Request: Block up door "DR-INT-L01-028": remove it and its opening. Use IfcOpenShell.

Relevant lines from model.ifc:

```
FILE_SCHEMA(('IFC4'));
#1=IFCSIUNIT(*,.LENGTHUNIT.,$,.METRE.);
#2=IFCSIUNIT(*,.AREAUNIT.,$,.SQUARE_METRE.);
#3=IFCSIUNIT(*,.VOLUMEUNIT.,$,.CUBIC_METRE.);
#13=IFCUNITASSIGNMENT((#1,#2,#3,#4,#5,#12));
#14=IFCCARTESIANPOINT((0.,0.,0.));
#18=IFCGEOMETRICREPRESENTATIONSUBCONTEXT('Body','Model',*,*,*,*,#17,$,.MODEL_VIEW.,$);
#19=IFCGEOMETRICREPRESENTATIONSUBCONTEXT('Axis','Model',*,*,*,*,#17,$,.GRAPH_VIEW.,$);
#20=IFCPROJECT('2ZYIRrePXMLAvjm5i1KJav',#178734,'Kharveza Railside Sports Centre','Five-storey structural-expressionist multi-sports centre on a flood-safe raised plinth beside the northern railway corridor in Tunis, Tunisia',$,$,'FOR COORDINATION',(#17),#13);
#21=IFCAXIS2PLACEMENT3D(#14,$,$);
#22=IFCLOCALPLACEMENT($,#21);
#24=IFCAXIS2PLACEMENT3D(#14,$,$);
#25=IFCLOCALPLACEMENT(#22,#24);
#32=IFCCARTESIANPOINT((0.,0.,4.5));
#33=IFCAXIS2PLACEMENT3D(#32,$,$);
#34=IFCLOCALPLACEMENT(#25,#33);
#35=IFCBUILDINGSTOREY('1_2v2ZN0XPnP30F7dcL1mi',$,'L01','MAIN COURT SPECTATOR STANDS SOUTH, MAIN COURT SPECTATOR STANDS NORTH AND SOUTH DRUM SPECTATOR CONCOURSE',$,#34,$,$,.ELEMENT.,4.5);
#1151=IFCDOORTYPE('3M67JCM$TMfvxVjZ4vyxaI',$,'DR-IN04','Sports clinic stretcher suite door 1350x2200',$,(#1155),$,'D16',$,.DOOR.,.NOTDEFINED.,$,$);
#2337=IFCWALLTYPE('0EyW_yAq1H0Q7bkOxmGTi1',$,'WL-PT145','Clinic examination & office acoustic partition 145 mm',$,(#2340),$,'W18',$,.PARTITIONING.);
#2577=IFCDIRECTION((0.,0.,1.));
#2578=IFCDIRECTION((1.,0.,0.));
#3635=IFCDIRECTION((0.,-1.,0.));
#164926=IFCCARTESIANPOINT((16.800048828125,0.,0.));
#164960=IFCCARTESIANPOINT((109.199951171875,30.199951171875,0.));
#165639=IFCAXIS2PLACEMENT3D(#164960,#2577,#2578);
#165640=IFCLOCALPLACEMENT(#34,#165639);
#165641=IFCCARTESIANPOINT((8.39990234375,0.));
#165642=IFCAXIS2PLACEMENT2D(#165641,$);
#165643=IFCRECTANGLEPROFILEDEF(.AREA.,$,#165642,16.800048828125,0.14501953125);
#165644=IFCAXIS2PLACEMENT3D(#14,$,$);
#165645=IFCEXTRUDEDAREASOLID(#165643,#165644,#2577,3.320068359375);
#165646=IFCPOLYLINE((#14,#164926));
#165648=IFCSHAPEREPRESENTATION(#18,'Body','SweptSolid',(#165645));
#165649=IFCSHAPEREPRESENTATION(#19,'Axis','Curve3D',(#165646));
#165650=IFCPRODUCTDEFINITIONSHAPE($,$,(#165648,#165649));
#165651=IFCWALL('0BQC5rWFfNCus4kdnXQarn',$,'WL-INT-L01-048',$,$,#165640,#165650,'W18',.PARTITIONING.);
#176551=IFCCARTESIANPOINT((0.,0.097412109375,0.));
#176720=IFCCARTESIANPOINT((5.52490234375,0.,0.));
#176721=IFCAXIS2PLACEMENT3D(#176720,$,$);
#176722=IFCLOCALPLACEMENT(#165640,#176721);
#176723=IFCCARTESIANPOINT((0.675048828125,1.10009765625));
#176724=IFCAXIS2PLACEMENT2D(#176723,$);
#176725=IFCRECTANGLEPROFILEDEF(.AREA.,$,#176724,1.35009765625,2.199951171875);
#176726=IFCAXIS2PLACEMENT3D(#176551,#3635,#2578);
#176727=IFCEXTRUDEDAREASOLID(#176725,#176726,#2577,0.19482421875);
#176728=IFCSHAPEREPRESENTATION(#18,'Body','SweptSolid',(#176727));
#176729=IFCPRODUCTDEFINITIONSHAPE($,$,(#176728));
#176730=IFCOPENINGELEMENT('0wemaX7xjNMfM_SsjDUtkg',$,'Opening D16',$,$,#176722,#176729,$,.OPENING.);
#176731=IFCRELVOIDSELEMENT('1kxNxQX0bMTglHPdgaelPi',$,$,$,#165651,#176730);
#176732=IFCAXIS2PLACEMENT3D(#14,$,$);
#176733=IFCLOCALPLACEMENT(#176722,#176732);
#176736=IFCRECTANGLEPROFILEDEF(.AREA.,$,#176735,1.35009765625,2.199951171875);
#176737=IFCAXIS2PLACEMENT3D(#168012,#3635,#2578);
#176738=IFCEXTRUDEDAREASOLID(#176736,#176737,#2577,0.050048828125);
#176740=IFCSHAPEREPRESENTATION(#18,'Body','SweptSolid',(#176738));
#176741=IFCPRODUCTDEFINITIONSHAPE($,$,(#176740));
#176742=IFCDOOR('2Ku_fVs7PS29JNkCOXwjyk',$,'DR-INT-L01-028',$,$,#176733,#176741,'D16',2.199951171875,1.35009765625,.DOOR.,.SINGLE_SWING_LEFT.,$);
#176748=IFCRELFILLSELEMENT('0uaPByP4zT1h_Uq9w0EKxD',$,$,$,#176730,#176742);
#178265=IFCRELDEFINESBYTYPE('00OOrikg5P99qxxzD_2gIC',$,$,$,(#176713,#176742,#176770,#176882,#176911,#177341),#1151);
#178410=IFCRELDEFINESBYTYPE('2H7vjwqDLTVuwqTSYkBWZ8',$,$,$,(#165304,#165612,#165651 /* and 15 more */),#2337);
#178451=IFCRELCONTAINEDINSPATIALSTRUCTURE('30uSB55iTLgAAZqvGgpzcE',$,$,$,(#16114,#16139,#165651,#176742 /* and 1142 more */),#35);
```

```python
import ifcopenshell
import ifcopenshell.api.feature
import ifcopenshell.api.root
import ifcopenshell.geom
import ifcopenshell.util.shape

model = ifcopenshell.open("model.ifc")
settings = ifcopenshell.geom.settings()


def volume(element):
    """Net volume in cubic metres, openings subtracted."""
    shape = ifcopenshell.geom.create_shape(settings, element)
    return ifcopenshell.util.shape.get_volume(shape.geometry)


door = model.by_guid("2Ku_fVs7PS29JNkCOXwjyk")
opening = door.FillsVoids[0].RelatingOpeningElement
wall = opening.VoidsElements[0].RelatingBuildingElement
before = volume(wall)

ifcopenshell.api.root.remove_product(model, product=door)
ifcopenshell.api.feature.remove_feature(model, feature=opening)

after = volume(wall)

print(f"wall volume {before:.3f} -> {after:.3f} m3")

model.write("model-out.ifc")
```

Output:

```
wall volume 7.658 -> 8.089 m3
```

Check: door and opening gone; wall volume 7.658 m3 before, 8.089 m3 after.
